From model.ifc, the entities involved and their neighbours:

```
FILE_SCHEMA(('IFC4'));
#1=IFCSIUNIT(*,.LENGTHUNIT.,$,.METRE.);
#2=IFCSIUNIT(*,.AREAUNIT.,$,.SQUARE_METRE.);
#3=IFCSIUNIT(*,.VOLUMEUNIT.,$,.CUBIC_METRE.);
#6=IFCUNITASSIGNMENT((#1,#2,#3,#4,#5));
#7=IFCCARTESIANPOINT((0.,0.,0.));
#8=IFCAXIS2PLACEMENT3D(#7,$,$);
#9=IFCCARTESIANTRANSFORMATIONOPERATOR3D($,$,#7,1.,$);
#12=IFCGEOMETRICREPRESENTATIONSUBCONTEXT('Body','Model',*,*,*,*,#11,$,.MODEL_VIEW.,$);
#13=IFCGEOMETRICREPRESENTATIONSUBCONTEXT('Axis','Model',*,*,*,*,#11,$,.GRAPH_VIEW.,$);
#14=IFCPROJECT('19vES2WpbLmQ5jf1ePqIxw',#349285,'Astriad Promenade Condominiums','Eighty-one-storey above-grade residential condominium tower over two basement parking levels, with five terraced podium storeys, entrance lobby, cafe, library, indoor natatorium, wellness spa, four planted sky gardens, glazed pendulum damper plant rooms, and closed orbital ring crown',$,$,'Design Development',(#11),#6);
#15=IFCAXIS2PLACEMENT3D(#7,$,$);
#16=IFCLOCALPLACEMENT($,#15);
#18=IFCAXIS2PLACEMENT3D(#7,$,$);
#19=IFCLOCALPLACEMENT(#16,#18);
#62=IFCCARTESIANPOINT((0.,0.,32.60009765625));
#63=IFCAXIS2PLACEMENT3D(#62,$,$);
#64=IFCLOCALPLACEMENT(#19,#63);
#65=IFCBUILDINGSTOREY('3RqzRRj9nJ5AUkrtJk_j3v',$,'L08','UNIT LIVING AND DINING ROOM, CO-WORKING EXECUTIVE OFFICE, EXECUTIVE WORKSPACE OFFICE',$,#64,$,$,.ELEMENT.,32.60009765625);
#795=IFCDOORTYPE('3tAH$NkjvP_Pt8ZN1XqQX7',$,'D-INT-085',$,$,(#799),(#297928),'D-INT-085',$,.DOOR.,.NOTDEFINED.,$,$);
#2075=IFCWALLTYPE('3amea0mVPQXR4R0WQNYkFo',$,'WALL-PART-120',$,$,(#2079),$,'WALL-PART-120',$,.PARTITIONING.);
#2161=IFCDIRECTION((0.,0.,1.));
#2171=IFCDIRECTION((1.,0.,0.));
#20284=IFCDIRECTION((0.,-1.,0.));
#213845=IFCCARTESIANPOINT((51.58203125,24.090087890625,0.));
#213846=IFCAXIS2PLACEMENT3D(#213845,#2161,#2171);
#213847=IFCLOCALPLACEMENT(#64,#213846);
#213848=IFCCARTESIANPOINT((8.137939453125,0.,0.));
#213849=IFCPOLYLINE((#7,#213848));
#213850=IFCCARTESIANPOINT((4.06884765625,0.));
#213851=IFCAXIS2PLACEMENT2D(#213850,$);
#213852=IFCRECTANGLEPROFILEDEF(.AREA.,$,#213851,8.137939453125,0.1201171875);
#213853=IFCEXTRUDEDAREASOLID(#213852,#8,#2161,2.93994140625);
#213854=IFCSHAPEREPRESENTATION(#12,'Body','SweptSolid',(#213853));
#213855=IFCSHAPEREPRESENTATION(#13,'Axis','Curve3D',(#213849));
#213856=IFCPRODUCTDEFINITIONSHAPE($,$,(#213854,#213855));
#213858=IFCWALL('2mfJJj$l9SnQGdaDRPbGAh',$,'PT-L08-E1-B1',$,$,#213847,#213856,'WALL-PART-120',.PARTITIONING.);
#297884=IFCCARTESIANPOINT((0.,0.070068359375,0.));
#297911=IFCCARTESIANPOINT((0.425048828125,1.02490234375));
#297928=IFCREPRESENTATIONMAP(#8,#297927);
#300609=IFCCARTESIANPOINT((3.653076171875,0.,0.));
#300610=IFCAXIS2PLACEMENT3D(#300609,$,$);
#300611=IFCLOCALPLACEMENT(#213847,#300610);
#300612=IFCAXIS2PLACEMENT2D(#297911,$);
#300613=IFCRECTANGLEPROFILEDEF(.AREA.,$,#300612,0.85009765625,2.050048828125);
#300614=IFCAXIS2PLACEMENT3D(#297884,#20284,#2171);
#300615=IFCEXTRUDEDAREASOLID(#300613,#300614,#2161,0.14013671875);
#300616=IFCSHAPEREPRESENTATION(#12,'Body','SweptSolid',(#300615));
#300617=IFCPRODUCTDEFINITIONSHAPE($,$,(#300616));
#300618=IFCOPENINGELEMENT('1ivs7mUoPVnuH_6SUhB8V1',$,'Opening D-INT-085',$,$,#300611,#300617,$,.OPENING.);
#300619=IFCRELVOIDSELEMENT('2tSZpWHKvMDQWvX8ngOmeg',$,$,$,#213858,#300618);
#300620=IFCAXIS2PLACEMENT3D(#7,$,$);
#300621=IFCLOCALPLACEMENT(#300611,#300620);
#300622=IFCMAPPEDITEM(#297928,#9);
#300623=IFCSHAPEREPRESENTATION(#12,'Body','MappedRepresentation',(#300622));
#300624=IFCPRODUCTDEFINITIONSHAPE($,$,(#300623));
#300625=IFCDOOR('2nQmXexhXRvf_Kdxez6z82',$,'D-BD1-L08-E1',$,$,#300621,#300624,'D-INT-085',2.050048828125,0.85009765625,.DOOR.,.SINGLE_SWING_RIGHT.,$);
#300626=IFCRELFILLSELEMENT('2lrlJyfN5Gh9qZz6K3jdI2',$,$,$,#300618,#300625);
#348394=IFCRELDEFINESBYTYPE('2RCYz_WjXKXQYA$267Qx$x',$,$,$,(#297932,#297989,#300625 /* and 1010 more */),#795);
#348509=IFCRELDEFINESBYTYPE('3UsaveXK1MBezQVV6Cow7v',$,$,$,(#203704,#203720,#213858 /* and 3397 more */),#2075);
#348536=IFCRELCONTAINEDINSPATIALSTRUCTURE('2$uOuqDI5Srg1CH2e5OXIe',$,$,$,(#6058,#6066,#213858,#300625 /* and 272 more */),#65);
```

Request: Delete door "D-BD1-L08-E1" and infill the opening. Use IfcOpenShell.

```python
import ifcopenshell
import ifcopenshell.api.feature
import ifcopenshell.api.root
import ifcopenshell.geom
import ifcopenshell.util.shape

model = ifcopenshell.open("model.ifc")
settings = ifcopenshell.geom.settings()


def volume(element):
    """Net volume in cubic metres, openings subtracted."""
    shape = ifcopenshell.geom.create_shape(settings, element)
    return ifcopenshell.util.shape.get_volume(shape.geometry)


door = model.by_guid("2nQmXexhXRvf_Kdxez6z82")
opening = door.FillsVoids[0].RelatingOpeningElement
wall = opening.VoidsElements[0].RelatingBuildingElement
before = volume(wall)

ifcopenshell.api.root.remove_product(model, product=door)
ifcopenshell.api.feature.remove_feature(model, feature=opening)

after = volume(wall)

print(f"wall volume {before:.3f} -> {after:.3f} m3")

model.write("model_edited.ifc")
```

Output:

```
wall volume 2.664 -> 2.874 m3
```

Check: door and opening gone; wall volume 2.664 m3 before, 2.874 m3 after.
